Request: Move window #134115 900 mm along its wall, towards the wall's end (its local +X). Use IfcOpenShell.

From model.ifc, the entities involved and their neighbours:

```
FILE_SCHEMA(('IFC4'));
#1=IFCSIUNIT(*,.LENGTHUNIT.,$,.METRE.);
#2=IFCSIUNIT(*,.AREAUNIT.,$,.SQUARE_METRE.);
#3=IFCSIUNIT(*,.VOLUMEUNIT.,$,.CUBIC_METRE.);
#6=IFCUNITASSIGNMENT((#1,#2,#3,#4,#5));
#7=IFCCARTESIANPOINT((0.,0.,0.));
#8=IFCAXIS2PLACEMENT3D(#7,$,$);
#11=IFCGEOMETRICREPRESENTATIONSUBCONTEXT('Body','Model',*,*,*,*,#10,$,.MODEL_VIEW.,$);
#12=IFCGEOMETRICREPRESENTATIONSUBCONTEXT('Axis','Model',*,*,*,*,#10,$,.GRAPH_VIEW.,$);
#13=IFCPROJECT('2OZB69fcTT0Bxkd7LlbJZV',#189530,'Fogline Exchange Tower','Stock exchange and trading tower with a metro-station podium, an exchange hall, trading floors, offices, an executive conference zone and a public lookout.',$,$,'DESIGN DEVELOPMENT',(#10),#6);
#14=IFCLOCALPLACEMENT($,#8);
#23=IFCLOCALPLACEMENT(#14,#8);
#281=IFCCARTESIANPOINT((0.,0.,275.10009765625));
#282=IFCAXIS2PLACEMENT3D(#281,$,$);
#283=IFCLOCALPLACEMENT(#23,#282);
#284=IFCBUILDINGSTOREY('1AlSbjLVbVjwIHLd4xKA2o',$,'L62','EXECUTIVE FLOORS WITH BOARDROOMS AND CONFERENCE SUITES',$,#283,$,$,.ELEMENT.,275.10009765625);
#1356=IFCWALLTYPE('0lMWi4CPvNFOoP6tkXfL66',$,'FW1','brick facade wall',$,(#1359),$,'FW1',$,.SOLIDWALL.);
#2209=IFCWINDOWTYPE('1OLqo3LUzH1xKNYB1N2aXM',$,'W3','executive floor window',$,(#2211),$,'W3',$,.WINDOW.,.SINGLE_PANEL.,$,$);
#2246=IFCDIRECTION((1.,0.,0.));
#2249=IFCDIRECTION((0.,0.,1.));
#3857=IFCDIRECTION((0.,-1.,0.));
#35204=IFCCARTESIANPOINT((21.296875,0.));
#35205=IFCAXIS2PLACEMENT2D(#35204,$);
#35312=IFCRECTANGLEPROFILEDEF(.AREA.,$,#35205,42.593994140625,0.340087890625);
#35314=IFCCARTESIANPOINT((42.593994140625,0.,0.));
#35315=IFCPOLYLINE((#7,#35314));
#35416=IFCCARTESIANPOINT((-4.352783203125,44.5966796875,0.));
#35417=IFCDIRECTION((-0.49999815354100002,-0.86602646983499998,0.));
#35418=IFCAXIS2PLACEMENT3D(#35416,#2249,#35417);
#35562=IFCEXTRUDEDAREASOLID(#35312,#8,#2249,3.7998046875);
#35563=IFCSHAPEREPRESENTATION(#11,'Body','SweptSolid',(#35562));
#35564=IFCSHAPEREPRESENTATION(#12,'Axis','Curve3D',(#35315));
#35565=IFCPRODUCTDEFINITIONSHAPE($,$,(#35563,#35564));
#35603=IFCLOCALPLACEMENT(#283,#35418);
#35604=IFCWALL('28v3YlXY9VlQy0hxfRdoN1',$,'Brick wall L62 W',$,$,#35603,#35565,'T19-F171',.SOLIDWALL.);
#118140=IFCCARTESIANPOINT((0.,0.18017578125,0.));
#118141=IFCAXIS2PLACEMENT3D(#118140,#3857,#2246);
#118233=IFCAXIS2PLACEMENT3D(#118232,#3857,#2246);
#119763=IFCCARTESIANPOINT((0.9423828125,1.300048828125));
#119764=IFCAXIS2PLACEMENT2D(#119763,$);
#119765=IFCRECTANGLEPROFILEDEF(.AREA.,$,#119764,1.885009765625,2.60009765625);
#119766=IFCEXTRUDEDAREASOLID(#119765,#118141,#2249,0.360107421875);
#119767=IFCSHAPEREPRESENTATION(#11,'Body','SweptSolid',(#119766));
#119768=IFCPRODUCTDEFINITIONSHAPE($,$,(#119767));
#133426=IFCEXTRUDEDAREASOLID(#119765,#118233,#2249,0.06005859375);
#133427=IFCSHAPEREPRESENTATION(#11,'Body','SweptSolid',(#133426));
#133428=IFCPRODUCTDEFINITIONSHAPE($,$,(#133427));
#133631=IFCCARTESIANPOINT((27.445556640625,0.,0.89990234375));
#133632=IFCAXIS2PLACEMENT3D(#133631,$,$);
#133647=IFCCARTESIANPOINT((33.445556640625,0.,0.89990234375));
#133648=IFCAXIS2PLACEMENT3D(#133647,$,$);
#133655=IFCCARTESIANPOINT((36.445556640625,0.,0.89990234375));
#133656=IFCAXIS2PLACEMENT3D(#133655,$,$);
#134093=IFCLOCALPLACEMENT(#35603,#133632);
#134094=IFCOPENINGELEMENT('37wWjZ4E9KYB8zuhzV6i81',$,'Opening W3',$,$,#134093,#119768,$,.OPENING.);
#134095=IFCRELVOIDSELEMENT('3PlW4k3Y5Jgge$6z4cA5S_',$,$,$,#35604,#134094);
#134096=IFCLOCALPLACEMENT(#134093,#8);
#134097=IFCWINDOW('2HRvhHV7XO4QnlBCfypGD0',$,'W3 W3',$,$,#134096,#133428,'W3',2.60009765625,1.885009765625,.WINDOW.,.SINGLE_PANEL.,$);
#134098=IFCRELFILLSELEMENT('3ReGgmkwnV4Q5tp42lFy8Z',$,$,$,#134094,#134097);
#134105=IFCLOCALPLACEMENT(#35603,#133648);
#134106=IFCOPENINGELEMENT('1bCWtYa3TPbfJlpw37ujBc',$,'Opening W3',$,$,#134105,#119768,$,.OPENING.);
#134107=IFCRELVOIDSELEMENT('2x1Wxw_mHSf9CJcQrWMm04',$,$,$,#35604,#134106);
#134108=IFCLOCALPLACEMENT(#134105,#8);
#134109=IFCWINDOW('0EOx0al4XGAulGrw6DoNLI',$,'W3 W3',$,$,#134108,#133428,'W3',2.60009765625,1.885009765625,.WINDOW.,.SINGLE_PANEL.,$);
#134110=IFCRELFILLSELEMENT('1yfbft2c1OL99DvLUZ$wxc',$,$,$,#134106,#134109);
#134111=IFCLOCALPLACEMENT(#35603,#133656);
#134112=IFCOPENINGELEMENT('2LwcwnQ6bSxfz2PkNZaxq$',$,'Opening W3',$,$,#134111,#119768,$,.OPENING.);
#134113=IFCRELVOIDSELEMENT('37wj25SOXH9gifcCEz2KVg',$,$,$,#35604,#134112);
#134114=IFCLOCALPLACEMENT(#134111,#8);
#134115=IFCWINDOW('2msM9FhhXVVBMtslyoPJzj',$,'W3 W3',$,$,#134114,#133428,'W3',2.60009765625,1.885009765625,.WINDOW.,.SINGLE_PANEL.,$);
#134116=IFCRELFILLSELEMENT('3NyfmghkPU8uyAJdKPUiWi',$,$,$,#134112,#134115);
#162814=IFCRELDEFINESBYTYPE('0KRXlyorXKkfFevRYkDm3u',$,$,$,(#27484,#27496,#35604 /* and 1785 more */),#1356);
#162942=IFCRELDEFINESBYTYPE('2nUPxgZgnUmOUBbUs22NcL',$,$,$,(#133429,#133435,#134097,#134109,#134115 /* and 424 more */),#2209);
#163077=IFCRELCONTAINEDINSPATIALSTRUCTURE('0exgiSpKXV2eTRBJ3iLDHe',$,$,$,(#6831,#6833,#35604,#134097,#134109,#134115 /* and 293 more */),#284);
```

```python
import ifcopenshell
import ifcopenshell.api.geometry
import ifcopenshell.util.placement
import ifcopenshell.util.unit

model = ifcopenshell.open("model.ifc")
unit_scale = ifcopenshell.util.unit.calculate_unit_scale(model)

window = model.by_id(134115)
opening = window.FillsVoids[0].RelatingOpeningElement
wall = opening.VoidsElements[0].RelatingBuildingElement

wall_matrix = ifcopenshell.util.placement.get_local_placement(wall.ObjectPlacement)
shift = wall_matrix[:3, 0] * 0.9 / unit_scale
before = ifcopenshell.util.placement.get_local_placement(window.ObjectPlacement)[:3, 3].copy()

# The window is placed relative to its opening, so it follows when the opening moves.
matrix = ifcopenshell.util.placement.get_local_placement(opening.ObjectPlacement)
matrix[:3, 3] += shift
ifcopenshell.api.geometry.edit_object_placement(
    model, product=opening, matrix=matrix, is_si=False, should_transform_children=True
)

after = ifcopenshell.util.placement.get_local_placement(window.ObjectPlacement)[:3, 3]
print("window moved by", (after - before).round(3) + 0.0)

model.write("model_updated.ifc")
```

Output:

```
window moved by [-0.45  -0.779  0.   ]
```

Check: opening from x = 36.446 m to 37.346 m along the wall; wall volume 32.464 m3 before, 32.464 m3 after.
